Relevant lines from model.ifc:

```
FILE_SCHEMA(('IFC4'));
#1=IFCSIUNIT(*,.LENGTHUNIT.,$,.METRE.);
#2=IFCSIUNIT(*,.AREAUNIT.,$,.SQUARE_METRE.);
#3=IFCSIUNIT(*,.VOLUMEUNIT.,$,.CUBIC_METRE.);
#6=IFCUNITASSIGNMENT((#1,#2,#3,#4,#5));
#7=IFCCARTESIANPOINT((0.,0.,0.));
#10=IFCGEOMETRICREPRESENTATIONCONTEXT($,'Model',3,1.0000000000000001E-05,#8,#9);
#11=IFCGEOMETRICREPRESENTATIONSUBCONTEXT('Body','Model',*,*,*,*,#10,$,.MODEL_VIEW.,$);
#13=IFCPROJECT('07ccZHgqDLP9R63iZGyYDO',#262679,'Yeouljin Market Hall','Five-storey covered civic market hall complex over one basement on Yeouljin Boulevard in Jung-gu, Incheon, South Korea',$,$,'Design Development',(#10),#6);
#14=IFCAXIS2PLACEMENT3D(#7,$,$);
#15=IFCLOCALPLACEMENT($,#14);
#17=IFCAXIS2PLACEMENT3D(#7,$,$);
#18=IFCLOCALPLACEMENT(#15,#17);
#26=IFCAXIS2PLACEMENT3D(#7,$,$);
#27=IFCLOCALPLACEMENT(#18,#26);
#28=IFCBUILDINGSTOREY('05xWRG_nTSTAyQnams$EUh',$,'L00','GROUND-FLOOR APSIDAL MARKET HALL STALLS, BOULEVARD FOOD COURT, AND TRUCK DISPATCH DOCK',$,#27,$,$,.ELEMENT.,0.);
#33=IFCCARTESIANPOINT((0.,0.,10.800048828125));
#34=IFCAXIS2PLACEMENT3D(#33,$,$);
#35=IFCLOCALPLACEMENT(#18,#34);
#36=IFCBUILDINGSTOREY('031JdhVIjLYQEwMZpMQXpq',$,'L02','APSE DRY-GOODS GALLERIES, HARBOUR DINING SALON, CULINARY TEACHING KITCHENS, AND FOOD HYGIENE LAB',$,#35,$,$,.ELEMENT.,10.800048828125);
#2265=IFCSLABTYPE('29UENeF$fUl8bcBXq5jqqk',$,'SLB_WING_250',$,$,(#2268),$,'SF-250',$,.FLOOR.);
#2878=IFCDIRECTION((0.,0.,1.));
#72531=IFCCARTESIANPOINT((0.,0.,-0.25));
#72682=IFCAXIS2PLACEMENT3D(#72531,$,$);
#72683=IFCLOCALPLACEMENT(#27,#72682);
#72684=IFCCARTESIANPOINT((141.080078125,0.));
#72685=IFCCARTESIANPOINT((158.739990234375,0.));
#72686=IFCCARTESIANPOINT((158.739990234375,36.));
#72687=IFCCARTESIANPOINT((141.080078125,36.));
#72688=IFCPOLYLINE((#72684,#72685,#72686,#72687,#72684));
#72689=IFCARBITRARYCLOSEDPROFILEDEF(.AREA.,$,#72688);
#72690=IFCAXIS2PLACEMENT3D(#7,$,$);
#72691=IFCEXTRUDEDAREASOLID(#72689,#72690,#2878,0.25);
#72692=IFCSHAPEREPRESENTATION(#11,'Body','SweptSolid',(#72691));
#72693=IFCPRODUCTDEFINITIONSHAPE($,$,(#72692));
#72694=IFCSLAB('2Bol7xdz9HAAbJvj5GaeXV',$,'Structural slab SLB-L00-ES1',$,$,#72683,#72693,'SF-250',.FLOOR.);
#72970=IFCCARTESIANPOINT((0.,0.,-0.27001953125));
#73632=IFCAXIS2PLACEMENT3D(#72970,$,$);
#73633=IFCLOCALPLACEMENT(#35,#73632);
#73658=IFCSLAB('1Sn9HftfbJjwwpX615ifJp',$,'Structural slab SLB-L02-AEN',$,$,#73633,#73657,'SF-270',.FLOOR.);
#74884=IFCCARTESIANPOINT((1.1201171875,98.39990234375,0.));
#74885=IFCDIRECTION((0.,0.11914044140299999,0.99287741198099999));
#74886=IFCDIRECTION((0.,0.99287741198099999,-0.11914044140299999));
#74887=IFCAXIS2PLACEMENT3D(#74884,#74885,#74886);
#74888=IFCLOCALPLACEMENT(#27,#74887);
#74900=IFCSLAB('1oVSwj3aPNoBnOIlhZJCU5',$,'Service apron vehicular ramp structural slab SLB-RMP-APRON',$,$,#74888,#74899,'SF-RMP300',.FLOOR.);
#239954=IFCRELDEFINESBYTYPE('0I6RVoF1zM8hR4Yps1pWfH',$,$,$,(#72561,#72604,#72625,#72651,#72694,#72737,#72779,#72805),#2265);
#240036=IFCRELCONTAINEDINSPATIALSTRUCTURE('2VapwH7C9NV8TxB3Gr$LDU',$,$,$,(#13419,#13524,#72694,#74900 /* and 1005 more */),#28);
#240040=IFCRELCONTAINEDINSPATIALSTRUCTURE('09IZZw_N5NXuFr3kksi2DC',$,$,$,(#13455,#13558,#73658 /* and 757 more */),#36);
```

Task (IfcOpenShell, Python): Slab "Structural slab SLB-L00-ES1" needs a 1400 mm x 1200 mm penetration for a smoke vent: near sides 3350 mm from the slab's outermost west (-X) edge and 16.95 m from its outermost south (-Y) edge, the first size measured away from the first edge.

```python
import numpy as np
import ifcopenshell
import ifcopenshell.api.feature
import ifcopenshell.api.geometry
import ifcopenshell.api.root
import ifcopenshell.geom
import ifcopenshell.util.placement
import ifcopenshell.util.representation
import ifcopenshell.util.shape
import ifcopenshell.util.unit

model = ifcopenshell.open("model.ifc")
unit_scale = ifcopenshell.util.unit.calculate_unit_scale(model)
settings = ifcopenshell.geom.settings()


def volume(element):
    """Net volume in cubic metres, openings subtracted."""
    shape = ifcopenshell.geom.create_shape(settings, element)
    return ifcopenshell.util.shape.get_volume(shape.geometry)


slab = model.by_guid("2Bol7xdz9HAAbJvj5GaeXV")
before = volume(slab)

# Extent in the slab's own axes, in metres. The edges named are its -X and -Y sides.
slab_shape = ifcopenshell.geom.create_shape(settings, slab)
vertices = ifcopenshell.util.shape.get_vertices(slab_shape.geometry)
x_min, y_min, bottom = vertices.min(axis=0)
top = vertices[:, 2].max()

opening = ifcopenshell.api.root.create_entity(model, ifc_class="IfcOpeningElement", name="Smoke vent opening", predefined_type="OPENING")
context = ifcopenshell.util.representation.get_context(model, "Model", "Body", "MODEL_VIEW")
width, depth = 1.4, 1.2
outline = [(0.0, 0.0), (width, 0.0), (width, depth), (0.0, depth), (0.0, 0.0)]
# Overshoot both faces by 50 mm so the cut is clean.
shape = ifcopenshell.api.geometry.add_slab_representation(
    model, context=context, depth=top - bottom + 0.1, polyline=outline
)
ifcopenshell.api.geometry.assign_representation(model, product=opening, representation=shape)

matrix = ifcopenshell.util.placement.get_local_placement(slab.ObjectPlacement)
matrix[:, 3] = matrix @ np.append(np.array([x_min + 3.35, y_min + 16.95, bottom - 0.05]) / unit_scale, 1.0)
ifcopenshell.api.geometry.edit_object_placement(model, product=opening, matrix=matrix, is_si=False)
ifcopenshell.api.feature.add_feature(model, feature=opening, element=slab)

after = volume(slab)

print(f"slab volume {before:.3f} -> {after:.3f} m3")

model.write("model_rev.ifc")
```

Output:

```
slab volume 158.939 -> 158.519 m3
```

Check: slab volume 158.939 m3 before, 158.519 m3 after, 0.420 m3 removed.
